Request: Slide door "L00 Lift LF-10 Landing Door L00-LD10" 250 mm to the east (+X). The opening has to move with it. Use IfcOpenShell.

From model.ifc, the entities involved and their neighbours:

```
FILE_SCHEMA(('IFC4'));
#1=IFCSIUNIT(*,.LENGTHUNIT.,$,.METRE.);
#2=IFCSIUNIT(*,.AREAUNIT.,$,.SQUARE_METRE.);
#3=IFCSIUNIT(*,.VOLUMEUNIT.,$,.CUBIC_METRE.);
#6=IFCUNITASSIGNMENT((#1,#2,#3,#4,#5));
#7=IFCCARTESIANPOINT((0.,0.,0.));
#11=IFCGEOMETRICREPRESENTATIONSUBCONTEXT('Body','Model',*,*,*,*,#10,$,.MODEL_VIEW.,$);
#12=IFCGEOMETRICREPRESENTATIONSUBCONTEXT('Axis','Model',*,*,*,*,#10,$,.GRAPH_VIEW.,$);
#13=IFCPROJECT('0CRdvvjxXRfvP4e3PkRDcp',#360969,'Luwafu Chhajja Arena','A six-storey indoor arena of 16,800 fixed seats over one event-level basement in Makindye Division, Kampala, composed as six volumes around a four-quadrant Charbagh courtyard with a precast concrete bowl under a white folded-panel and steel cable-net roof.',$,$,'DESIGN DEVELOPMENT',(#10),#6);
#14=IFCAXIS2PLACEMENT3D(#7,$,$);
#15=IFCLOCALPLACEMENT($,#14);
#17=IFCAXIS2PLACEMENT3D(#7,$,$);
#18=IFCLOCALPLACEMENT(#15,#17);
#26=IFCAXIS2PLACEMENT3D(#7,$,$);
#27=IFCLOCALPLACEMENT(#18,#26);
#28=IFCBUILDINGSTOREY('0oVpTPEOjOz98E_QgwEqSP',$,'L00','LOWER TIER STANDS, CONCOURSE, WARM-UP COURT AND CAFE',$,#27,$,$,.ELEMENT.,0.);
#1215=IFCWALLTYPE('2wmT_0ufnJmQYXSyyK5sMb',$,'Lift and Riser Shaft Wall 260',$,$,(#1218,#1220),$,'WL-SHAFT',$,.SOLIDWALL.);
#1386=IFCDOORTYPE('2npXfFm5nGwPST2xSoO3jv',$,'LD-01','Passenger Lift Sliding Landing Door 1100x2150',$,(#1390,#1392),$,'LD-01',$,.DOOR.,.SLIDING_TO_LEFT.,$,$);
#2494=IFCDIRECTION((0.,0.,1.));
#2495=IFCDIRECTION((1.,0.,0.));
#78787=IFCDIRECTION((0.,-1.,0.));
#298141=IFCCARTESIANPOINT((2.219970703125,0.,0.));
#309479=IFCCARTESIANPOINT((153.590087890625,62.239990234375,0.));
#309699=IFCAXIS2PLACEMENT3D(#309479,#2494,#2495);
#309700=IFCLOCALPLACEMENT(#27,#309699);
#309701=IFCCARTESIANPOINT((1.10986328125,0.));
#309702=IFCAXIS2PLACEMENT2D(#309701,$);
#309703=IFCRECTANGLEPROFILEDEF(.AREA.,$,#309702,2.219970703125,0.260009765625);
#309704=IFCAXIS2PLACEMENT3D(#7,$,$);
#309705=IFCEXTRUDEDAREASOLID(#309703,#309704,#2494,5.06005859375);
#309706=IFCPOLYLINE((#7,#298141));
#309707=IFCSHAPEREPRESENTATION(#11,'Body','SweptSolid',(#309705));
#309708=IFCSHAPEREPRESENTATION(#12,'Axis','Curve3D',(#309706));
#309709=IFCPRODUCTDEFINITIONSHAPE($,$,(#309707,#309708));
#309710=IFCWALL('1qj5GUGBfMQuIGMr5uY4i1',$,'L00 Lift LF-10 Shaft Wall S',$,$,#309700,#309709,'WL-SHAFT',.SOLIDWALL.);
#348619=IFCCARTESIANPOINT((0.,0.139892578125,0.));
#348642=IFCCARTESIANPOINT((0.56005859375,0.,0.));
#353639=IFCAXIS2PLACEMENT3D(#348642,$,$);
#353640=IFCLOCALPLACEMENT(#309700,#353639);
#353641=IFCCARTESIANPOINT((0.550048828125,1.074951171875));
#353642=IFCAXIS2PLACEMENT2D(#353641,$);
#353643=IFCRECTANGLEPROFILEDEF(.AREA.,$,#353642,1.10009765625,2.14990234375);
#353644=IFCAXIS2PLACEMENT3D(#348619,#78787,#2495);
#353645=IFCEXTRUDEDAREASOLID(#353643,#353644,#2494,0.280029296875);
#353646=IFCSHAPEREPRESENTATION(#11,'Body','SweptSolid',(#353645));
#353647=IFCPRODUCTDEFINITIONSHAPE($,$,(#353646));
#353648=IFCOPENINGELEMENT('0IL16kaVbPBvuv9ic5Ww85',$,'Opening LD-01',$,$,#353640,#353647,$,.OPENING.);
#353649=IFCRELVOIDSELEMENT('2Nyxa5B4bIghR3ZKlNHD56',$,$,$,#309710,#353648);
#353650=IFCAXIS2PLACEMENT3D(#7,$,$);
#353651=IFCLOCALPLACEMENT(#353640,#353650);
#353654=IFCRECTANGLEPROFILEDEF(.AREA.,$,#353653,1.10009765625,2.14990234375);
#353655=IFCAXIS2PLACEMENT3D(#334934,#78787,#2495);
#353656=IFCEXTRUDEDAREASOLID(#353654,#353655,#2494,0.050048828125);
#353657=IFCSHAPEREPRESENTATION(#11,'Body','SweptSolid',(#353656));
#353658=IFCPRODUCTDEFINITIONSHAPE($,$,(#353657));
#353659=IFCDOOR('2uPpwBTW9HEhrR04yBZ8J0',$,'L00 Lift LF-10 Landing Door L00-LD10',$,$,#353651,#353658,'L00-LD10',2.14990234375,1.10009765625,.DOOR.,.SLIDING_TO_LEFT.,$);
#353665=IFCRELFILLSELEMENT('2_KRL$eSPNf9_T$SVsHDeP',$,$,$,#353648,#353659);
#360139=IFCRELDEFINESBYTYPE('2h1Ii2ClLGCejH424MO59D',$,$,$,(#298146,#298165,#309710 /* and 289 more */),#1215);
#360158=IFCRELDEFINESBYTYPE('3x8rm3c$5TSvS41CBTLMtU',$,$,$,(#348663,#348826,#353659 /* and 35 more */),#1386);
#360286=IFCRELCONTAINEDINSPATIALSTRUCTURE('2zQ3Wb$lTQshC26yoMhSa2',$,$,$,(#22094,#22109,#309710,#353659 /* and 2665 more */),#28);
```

```python
import ifcopenshell
import ifcopenshell.api.geometry
import ifcopenshell.util.placement
import ifcopenshell.util.unit

model = ifcopenshell.open("model.ifc")
unit_scale = ifcopenshell.util.unit.calculate_unit_scale(model)

door = model.by_guid("2uPpwBTW9HEhrR04yBZ8J0")
opening = door.FillsVoids[0].RelatingOpeningElement
wall = opening.VoidsElements[0].RelatingBuildingElement

wall_matrix = ifcopenshell.util.placement.get_local_placement(wall.ObjectPlacement)
shift = wall_matrix[:3, 0] * 0.25 / unit_scale
before = ifcopenshell.util.placement.get_local_placement(door.ObjectPlacement)[:3, 3].copy()

# The door is placed relative to its opening, so it follows when the opening moves.
matrix = ifcopenshell.util.placement.get_local_placement(opening.ObjectPlacement)
matrix[:3, 3] += shift
ifcopenshell.api.geometry.edit_object_placement(
    model, product=opening, matrix=matrix, is_si=False, should_transform_children=True
)

after = ifcopenshell.util.placement.get_local_placement(door.ObjectPlacement)[:3, 3]
print("door moved by", (after - before).round(3) + 0.0)

model.write("model-out.ifc")
```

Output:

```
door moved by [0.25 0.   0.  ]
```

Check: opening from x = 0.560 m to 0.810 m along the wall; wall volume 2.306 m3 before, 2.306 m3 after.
